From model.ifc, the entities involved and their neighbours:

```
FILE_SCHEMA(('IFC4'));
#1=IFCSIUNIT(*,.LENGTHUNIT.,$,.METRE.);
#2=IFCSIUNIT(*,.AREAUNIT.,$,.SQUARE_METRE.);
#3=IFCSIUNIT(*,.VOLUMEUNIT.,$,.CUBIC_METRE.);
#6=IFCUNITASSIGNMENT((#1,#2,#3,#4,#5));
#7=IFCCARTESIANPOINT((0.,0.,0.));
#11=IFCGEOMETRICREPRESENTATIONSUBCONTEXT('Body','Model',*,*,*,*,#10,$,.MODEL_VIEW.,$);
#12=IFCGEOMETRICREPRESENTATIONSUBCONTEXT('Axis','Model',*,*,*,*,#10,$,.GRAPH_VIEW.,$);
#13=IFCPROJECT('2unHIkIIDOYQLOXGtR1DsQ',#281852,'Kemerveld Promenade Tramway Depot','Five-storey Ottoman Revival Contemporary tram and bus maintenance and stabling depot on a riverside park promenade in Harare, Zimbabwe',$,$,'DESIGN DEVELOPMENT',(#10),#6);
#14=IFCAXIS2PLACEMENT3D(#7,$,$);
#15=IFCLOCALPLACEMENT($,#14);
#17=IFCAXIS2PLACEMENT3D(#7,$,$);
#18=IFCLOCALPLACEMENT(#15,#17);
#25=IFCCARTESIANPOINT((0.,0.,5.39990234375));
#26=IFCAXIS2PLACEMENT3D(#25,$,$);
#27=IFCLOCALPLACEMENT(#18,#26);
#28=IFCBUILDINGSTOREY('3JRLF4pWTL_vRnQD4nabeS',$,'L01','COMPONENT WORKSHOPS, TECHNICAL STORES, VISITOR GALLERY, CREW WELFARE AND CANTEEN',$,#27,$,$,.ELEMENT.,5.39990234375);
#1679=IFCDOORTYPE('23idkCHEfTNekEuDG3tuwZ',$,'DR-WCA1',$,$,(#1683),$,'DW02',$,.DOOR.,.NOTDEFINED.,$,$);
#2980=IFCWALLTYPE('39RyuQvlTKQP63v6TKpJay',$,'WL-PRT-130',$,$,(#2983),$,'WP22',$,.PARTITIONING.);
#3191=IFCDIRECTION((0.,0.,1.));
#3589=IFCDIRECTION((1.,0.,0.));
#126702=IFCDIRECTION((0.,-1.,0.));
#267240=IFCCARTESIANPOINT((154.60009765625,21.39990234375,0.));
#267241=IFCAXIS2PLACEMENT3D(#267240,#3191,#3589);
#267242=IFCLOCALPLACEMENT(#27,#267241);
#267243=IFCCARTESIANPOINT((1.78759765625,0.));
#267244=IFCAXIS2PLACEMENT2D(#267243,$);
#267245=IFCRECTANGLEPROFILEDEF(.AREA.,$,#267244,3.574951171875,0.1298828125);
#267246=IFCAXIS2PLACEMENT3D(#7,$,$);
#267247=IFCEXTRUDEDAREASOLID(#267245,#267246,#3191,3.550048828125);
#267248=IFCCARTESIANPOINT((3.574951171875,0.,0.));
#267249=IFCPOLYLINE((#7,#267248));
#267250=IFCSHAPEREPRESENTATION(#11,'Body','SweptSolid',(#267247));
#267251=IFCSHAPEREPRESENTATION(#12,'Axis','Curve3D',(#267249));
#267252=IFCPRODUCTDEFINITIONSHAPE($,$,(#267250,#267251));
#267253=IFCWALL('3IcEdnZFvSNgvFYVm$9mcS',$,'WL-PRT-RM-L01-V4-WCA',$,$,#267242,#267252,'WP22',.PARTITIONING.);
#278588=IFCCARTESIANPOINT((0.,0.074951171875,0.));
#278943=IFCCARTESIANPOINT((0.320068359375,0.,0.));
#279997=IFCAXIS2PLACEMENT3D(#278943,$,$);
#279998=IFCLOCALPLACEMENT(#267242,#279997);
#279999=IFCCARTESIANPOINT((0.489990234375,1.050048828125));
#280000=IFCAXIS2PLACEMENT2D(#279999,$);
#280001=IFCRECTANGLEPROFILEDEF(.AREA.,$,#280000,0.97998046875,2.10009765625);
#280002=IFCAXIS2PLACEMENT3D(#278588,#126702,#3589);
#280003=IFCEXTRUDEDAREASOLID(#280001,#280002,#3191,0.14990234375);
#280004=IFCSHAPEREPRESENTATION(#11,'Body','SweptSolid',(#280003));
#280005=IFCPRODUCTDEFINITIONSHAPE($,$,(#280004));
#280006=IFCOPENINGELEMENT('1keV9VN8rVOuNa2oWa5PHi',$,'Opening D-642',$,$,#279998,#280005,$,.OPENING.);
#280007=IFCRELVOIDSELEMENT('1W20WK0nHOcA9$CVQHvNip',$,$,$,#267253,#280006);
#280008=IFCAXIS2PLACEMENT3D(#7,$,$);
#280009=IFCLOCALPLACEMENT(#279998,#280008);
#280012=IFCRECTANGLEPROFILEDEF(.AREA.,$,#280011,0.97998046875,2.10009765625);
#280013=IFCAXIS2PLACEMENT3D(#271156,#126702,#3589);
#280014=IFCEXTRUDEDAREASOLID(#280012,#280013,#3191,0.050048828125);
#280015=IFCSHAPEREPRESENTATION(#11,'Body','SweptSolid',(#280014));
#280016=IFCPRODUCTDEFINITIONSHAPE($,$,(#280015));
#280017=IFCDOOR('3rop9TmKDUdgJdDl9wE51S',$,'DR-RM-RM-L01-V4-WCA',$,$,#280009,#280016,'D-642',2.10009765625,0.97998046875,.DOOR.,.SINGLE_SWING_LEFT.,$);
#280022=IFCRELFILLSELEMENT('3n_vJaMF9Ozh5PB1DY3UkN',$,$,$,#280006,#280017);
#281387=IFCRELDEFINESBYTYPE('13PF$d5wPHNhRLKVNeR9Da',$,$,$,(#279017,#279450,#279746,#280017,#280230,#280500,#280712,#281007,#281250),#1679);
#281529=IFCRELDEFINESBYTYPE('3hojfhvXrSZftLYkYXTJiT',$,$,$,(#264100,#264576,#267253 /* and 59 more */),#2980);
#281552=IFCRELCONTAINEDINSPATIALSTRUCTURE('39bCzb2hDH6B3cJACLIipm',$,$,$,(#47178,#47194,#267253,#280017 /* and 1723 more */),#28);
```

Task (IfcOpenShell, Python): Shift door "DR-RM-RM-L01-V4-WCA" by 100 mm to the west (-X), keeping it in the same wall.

```python
import ifcopenshell
import ifcopenshell.api.geometry
import ifcopenshell.util.placement
import ifcopenshell.util.unit

model = ifcopenshell.open("model.ifc")
unit_scale = ifcopenshell.util.unit.calculate_unit_scale(model)

door = model.by_id(280017)
opening = door.FillsVoids[0].RelatingOpeningElement
wall = opening.VoidsElements[0].RelatingBuildingElement

wall_matrix = ifcopenshell.util.placement.get_local_placement(wall.ObjectPlacement)
shift = wall_matrix[:3, 0] * -0.1 / unit_scale
before = ifcopenshell.util.placement.get_local_placement(door.ObjectPlacement)[:3, 3].copy()

# The door is placed relative to its opening, so it follows when the opening moves.
matrix = ifcopenshell.util.placement.get_local_placement(opening.ObjectPlacement)
matrix[:3, 3] += shift
ifcopenshell.api.geometry.edit_object_placement(
    model, product=opening, matrix=matrix, is_si=False, should_transform_children=True
)

after = ifcopenshell.util.placement.get_local_placement(door.ObjectPlacement)[:3, 3]
print("door moved by", (after - before).round(3) + 0.0)

model.write("model_edited.ifc")
```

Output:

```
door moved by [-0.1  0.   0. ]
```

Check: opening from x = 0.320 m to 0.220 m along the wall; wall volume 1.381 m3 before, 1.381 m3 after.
